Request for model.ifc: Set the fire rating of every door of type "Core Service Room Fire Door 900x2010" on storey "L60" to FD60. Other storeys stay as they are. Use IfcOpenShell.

First a look at what the model holds.

```python
import ifcopenshell
import ifcopenshell.util.element

model = ifcopenshell.open("model.ifc")
print(model.schema)
storey = next(s for s in model.by_type("IfcBuildingStorey") if s.Name == "L60")
doors = [e for e in ifcopenshell.util.element.get_decomposition(storey) if e.is_a("IfcDoor")]
seen = {}
for e in doors:
    element_type = ifcopenshell.util.element.get_type(e)
    key = (element_type.Name if element_type != e and element_type else None, ifcopenshell.util.element.get_pset(e, "Pset_DoorCommon", "FireRating"))
    seen[key] = seen.get(key, 0) + 1
for (name, value), count in sorted(seen.items(), key=str):
    print(count, "x", name, "|", value)
```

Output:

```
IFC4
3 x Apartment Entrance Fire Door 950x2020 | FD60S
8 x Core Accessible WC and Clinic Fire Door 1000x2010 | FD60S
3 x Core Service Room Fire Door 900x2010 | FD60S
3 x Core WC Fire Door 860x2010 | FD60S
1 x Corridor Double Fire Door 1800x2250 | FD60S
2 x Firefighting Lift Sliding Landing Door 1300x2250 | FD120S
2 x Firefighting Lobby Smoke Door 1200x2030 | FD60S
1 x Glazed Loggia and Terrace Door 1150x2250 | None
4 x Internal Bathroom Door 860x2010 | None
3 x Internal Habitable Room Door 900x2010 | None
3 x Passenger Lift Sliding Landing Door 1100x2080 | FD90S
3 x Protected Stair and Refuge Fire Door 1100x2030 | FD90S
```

```python
import ifcopenshell
import ifcopenshell.api.pset
import ifcopenshell.util.element

model = ifcopenshell.open("model.ifc")

storey = next(s for s in model.by_type("IfcBuildingStorey") if s.Name == "L60")
doors = [e for e in ifcopenshell.util.element.get_decomposition(storey) if e.is_a("IfcDoor")]

count = 0
for e in doors:
    element_type = ifcopenshell.util.element.get_type(e)
    if element_type in (None, e) or element_type.Name != "Core Service Room Fire Door 900x2010":
        continue
    found = ifcopenshell.util.element.get_pset(e, "Pset_DoorCommon", should_inherit=False)
    if found:
        pset = model.by_id(found["id"])
        if len(ifcopenshell.util.element.get_elements_by_pset(pset)) > 1:
            pset = ifcopenshell.api.pset.unshare_pset(model, products=[e], pset=pset)[0]
    else:
        pset = ifcopenshell.api.pset.add_pset(model, product=e, name="Pset_DoorCommon")
    ifcopenshell.api.pset.edit_pset(model, pset=pset, properties={"FireRating": "FD60"})
    count += 1

print(count, "doors updated")

model.write("model_edited.ifc")
```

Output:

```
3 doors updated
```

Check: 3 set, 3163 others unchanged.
